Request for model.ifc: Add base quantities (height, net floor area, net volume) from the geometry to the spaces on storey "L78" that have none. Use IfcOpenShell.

First a look at what the model holds.

```python
import ifcopenshell
import ifcopenshell.util.element
import ifcopenshell.util.unit

model = ifcopenshell.open("model.ifc")
print(model.schema)
for unit_type in ("LENGTHUNIT", "AREAUNIT", "VOLUMEUNIT"):
    print(unit_type, ifcopenshell.util.unit.calculate_unit_scale(model, unit_type))
storey = next(s for s in model.by_type("IfcBuildingStorey") if s.Name == "L78")
spaces = [e for e in ifcopenshell.util.element.get_decomposition(storey) if e.is_a("IfcSpace")]
for e in sorted(spaces, key=lambda e: e.id()):
    print(e.id(), e.is_a(), e.Name, list(ifcopenshell.util.element.get_psets(e, qtos_only=True)), sep=" | ")
```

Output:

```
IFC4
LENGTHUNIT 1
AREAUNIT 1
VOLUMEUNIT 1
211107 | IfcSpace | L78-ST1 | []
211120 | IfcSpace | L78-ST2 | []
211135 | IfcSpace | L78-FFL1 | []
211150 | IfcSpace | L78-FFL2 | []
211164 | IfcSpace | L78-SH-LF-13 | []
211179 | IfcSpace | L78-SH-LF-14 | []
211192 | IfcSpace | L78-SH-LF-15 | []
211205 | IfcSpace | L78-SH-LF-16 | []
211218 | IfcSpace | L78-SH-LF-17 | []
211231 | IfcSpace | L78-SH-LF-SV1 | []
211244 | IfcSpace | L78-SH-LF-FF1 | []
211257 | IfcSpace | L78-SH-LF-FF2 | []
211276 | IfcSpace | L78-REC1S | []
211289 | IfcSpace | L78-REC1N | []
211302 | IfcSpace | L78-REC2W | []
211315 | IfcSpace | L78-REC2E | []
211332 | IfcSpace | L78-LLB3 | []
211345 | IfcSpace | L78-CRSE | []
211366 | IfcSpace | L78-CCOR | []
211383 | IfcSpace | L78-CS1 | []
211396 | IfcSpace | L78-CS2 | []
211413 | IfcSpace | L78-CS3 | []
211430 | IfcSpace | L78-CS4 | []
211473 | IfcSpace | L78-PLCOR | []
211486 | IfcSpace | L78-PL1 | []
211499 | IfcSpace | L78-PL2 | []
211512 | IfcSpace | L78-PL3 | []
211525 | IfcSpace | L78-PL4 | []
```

```python
import ifcopenshell
import ifcopenshell.api.pset
import ifcopenshell.geom
import ifcopenshell.util.element
import ifcopenshell.util.shape
import ifcopenshell.util.unit

model = ifcopenshell.open("model.ifc")
unit_scale = ifcopenshell.util.unit.calculate_unit_scale(model)
area_scale = ifcopenshell.util.unit.calculate_unit_scale(model, "AREAUNIT")
volume_scale = ifcopenshell.util.unit.calculate_unit_scale(model, "VOLUMEUNIT")
settings = ifcopenshell.geom.settings()

storey = next(s for s in model.by_type("IfcBuildingStorey") if s.Name == "L78")
spaces = [e for e in ifcopenshell.util.element.get_decomposition(storey) if e.is_a("IfcSpace")]

for e in sorted(spaces, key=lambda e: e.id()):
    if ifcopenshell.util.element.get_psets(e, qtos_only=True, should_inherit=False):
        continue
    # Geometry comes back in metres, in the element's own axes.
    shape = ifcopenshell.geom.create_shape(settings, e)
    values = {
        "Height": ifcopenshell.util.shape.get_z(shape.geometry) / unit_scale,
        "NetFloorArea": ifcopenshell.util.shape.get_footprint_area(shape.geometry) / area_scale,
        "NetVolume": ifcopenshell.util.shape.get_volume(shape.geometry) / volume_scale,
    }
    qto = ifcopenshell.api.pset.add_qto(model, product=e, name="Qto_SpaceBaseQuantities")
    ifcopenshell.api.pset.edit_qto(model, qto=qto, properties=values)
    print(e.id(), {k: round(v, 3) for k, v in values.items()})

model.write("model_edited.ifc")
```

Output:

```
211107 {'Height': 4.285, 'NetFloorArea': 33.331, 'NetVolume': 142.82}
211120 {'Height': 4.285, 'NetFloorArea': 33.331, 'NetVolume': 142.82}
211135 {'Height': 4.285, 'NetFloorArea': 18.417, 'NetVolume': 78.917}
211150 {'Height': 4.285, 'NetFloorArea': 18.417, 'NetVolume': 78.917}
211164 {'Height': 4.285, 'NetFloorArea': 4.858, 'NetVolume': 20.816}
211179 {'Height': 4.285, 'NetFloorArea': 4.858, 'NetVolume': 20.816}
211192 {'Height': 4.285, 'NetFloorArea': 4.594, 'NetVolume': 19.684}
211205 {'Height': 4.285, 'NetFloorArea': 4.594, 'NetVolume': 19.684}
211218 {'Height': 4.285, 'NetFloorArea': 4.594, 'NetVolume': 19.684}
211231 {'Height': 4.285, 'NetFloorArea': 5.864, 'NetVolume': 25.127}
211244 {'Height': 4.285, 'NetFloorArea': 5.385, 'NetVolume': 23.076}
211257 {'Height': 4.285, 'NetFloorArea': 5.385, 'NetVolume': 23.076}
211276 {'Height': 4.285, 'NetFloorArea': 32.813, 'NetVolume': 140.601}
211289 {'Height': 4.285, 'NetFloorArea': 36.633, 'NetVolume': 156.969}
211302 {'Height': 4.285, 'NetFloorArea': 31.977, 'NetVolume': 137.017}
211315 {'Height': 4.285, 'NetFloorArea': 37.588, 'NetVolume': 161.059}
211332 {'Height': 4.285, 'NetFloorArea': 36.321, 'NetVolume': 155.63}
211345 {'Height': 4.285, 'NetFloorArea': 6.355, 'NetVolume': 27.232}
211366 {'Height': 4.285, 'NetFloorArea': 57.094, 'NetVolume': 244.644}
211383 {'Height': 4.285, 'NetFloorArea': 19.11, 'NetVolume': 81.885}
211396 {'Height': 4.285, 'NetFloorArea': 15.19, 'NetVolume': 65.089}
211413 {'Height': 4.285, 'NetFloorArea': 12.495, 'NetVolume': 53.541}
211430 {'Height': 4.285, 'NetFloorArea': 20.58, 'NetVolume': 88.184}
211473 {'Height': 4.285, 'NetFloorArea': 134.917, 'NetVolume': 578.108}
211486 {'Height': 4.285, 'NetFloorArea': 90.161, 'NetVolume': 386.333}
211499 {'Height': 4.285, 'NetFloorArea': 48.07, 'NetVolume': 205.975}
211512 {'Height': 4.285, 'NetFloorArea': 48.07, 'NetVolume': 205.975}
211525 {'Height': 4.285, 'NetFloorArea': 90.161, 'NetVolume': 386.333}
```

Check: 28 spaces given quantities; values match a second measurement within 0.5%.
